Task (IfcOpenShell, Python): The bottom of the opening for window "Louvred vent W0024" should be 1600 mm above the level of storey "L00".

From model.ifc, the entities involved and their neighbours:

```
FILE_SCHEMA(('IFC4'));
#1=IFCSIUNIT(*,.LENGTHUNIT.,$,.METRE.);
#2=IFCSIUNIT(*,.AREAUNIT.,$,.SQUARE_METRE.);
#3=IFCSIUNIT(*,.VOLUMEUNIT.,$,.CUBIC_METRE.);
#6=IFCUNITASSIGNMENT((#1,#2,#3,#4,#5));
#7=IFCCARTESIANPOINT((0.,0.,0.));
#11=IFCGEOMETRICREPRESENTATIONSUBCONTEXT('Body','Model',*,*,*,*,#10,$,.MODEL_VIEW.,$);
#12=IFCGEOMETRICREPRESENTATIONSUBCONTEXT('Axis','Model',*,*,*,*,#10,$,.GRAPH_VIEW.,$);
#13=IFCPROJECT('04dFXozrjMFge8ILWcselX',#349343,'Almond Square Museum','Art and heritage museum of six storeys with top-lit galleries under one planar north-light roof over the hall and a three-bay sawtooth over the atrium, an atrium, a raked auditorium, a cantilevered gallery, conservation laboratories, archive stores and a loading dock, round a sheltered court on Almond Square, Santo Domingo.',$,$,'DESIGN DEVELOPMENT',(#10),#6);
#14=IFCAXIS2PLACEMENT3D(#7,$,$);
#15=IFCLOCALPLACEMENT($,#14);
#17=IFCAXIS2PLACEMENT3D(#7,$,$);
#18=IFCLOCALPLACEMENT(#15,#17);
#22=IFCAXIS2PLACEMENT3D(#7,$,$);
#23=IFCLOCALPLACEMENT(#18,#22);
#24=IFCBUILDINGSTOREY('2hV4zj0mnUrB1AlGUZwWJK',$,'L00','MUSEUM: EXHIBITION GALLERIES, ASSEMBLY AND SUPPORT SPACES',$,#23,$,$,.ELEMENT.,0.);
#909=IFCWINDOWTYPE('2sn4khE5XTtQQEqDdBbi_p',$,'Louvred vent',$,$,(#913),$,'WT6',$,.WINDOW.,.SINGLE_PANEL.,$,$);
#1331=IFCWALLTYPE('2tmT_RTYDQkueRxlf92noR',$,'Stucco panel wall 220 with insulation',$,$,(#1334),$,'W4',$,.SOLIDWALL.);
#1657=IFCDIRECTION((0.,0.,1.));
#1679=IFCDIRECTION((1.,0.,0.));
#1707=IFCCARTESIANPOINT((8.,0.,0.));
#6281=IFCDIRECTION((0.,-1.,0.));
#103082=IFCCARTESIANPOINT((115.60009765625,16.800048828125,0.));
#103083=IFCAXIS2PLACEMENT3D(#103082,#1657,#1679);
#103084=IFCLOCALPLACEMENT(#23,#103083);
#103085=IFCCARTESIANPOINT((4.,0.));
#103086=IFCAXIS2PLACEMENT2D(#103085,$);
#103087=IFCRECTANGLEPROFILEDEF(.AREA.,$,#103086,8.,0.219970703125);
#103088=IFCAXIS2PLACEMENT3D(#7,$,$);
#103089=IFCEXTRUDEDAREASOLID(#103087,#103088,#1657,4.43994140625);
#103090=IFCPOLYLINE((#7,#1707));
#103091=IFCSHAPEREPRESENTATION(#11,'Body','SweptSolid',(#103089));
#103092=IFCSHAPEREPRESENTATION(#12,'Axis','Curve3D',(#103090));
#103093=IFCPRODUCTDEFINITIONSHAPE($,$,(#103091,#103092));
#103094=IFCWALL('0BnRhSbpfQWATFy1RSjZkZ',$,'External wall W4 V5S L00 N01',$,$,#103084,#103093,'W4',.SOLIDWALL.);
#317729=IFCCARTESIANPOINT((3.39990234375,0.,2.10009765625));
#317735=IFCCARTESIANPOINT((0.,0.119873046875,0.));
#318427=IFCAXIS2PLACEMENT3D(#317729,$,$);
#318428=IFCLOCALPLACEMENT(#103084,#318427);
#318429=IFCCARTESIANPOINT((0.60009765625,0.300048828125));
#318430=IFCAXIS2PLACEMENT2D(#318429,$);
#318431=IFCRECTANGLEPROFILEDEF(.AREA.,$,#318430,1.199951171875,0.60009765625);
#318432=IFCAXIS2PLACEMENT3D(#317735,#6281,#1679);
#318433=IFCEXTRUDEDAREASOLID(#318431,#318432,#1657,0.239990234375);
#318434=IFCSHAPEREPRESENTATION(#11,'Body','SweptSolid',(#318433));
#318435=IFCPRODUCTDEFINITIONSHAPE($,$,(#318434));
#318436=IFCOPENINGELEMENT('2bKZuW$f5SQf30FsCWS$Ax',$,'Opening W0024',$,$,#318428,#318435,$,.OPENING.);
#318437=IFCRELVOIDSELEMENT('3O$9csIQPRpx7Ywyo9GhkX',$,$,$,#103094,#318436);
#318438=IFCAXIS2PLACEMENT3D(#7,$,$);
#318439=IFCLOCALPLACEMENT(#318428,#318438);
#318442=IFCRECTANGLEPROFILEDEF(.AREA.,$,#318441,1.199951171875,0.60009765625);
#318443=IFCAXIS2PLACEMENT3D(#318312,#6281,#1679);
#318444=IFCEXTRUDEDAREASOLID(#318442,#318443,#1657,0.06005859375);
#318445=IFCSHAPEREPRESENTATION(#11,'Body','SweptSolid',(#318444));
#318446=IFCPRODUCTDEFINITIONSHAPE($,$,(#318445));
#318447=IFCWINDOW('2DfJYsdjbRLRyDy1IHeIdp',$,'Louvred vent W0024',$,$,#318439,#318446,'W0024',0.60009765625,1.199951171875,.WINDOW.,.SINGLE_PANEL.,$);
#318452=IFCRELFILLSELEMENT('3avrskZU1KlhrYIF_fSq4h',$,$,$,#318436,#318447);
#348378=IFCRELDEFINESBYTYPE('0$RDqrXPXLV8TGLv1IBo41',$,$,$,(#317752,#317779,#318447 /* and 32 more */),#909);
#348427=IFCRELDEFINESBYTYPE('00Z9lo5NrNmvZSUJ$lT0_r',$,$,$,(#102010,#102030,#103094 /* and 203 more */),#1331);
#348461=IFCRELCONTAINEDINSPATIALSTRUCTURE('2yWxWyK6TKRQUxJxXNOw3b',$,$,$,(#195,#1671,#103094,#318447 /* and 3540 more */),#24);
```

```python
import numpy as np
import ifcopenshell
import ifcopenshell.api.geometry
import ifcopenshell.geom
import ifcopenshell.util.element
import ifcopenshell.util.placement
import ifcopenshell.util.shape
import ifcopenshell.util.unit

model = ifcopenshell.open("model.ifc")
unit_scale = ifcopenshell.util.unit.calculate_unit_scale(model)

window = model.by_id(318447)
opening = window.FillsVoids[0].RelatingOpeningElement
storey = ifcopenshell.util.element.get_container(window, ifc_class="IfcBuildingStorey")
level = ifcopenshell.util.placement.get_local_placement(storey.ObjectPlacement)[2, 3]

# The opening's origin need not be at the sill, so measure its lowest point.
shape = ifcopenshell.geom.create_shape(ifcopenshell.geom.settings(), opening)
bottom = ifcopenshell.util.shape.get_shape_bottom_elevation(shape, shape.geometry) / unit_scale
dz = level + 1.6 / unit_scale - bottom

shift = np.array([0.0, 0.0, dz])
# The window is placed relative to its opening, so it follows when the opening moves.
matrix = ifcopenshell.util.placement.get_local_placement(opening.ObjectPlacement)
matrix[:3, 3] += shift
ifcopenshell.api.geometry.edit_object_placement(
    model, product=opening, matrix=matrix, is_si=False, should_transform_children=True
)

print(f"moved by {dz * unit_scale:+.3f} m")

model.write("model_updated.ifc")
```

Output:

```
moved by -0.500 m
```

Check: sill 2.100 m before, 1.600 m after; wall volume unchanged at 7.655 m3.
